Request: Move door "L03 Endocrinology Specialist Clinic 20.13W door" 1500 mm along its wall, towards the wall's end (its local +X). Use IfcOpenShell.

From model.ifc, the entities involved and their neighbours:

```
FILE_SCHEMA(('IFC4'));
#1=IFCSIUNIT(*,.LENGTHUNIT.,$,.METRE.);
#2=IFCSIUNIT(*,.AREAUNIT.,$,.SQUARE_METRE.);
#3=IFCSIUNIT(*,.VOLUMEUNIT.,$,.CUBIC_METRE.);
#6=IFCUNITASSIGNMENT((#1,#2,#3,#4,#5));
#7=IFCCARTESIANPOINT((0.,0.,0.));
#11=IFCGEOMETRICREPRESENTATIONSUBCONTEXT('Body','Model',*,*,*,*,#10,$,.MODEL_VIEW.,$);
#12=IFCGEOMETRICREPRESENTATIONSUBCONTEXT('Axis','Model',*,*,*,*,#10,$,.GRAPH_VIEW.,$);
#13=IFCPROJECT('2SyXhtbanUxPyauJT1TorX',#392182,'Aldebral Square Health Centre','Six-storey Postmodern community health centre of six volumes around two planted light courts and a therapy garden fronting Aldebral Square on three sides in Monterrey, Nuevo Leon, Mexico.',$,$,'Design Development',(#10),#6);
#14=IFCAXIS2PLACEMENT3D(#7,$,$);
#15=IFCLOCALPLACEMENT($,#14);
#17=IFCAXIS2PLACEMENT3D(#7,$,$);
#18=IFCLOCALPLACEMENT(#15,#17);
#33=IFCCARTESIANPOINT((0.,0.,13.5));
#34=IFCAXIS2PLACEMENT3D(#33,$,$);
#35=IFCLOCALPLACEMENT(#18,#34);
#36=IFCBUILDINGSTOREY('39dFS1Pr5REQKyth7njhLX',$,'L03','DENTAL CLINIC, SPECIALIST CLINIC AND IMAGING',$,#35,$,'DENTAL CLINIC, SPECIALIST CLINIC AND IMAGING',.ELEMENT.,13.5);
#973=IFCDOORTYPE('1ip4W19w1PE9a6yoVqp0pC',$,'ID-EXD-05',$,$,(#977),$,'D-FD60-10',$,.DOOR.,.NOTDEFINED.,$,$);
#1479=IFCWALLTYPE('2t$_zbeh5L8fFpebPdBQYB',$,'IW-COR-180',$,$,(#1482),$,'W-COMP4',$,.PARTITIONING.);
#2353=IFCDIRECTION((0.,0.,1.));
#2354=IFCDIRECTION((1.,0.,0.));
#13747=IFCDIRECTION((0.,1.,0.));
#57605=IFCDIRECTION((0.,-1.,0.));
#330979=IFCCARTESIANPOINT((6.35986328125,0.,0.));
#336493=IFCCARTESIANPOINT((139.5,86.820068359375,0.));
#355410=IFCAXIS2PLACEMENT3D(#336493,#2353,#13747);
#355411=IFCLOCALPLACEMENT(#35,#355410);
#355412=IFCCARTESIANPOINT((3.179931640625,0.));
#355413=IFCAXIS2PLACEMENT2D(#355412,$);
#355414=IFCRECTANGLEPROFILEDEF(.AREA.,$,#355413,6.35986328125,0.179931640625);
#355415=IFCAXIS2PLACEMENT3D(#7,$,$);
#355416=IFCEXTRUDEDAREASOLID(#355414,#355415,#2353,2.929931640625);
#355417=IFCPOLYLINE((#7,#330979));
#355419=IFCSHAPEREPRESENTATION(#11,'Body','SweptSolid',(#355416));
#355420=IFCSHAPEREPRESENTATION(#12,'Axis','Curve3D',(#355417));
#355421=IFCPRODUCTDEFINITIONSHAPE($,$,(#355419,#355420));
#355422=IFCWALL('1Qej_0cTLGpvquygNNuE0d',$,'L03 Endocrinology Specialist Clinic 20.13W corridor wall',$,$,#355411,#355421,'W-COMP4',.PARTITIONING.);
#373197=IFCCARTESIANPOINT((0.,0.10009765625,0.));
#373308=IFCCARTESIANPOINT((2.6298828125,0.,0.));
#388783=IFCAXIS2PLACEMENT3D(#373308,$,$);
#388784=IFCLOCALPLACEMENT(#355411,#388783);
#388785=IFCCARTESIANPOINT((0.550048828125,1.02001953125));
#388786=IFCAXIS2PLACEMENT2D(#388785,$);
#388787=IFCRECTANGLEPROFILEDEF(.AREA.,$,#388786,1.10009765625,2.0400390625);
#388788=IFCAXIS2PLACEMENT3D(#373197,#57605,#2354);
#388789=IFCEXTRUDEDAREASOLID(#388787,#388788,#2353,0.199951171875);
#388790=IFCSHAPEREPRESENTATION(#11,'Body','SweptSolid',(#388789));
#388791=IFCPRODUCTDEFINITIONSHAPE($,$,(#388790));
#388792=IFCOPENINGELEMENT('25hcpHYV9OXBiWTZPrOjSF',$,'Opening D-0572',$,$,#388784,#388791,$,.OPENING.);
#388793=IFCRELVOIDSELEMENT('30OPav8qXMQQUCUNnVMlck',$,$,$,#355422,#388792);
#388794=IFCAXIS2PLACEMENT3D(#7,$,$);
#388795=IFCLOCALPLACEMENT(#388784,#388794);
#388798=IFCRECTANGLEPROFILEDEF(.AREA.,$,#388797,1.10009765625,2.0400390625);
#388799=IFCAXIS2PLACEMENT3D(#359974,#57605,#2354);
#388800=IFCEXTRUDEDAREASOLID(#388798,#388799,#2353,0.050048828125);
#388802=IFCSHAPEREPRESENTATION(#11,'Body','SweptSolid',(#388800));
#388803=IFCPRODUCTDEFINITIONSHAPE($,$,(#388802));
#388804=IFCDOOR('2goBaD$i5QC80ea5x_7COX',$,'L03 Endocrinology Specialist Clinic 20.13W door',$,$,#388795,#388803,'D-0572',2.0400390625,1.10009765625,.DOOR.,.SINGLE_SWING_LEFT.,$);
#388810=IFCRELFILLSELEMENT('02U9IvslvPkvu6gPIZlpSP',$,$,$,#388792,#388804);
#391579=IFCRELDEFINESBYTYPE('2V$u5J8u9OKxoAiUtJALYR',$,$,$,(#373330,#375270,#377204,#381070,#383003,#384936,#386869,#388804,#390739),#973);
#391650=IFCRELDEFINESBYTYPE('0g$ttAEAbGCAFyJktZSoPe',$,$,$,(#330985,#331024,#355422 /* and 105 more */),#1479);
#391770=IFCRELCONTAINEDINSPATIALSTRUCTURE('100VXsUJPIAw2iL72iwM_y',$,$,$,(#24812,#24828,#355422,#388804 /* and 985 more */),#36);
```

```python
import ifcopenshell
import ifcopenshell.api.geometry
import ifcopenshell.util.placement
import ifcopenshell.util.unit

model = ifcopenshell.open("model.ifc")
unit_scale = ifcopenshell.util.unit.calculate_unit_scale(model)

door = model.by_guid("2goBaD$i5QC80ea5x_7COX")
opening = door.FillsVoids[0].RelatingOpeningElement
wall = opening.VoidsElements[0].RelatingBuildingElement

wall_matrix = ifcopenshell.util.placement.get_local_placement(wall.ObjectPlacement)
shift = wall_matrix[:3, 0] * 1.5 / unit_scale
before = ifcopenshell.util.placement.get_local_placement(door.ObjectPlacement)[:3, 3].copy()

# The door is placed relative to its opening, so it follows when the opening moves.
matrix = ifcopenshell.util.placement.get_local_placement(opening.ObjectPlacement)
matrix[:3, 3] += shift
ifcopenshell.api.geometry.edit_object_placement(
    model, product=opening, matrix=matrix, is_si=False, should_transform_children=True
)

after = ifcopenshell.util.placement.get_local_placement(door.ObjectPlacement)[:3, 3]
print("door moved by", (after - before).round(3) + 0.0)

model.write("model_rev.ifc")
```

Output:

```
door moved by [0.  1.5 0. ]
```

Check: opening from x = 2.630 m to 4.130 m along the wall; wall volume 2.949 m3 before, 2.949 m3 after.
